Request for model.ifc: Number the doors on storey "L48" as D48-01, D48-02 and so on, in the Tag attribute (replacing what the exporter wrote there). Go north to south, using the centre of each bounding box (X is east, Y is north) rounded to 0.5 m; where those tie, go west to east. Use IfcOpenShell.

First a look at what the model holds.

```python
import ifcopenshell
import ifcopenshell.util.element
import ifcopenshell.util.placement

model = ifcopenshell.open("model.ifc")
print(model.schema)
storey = next(s for s in model.by_type("IfcBuildingStorey") if s.Name == "L48")
doors = [e for e in ifcopenshell.util.element.get_decomposition(storey) if e.is_a("IfcDoor")]
for e in sorted(doors, key=lambda e: e.id()):
    origin = ifcopenshell.util.placement.get_local_placement(e.ObjectPlacement)[:3, 3]
    print(e.id(), e.Tag, e.Name, origin.round(2) + 0.0, sep=" | ")
```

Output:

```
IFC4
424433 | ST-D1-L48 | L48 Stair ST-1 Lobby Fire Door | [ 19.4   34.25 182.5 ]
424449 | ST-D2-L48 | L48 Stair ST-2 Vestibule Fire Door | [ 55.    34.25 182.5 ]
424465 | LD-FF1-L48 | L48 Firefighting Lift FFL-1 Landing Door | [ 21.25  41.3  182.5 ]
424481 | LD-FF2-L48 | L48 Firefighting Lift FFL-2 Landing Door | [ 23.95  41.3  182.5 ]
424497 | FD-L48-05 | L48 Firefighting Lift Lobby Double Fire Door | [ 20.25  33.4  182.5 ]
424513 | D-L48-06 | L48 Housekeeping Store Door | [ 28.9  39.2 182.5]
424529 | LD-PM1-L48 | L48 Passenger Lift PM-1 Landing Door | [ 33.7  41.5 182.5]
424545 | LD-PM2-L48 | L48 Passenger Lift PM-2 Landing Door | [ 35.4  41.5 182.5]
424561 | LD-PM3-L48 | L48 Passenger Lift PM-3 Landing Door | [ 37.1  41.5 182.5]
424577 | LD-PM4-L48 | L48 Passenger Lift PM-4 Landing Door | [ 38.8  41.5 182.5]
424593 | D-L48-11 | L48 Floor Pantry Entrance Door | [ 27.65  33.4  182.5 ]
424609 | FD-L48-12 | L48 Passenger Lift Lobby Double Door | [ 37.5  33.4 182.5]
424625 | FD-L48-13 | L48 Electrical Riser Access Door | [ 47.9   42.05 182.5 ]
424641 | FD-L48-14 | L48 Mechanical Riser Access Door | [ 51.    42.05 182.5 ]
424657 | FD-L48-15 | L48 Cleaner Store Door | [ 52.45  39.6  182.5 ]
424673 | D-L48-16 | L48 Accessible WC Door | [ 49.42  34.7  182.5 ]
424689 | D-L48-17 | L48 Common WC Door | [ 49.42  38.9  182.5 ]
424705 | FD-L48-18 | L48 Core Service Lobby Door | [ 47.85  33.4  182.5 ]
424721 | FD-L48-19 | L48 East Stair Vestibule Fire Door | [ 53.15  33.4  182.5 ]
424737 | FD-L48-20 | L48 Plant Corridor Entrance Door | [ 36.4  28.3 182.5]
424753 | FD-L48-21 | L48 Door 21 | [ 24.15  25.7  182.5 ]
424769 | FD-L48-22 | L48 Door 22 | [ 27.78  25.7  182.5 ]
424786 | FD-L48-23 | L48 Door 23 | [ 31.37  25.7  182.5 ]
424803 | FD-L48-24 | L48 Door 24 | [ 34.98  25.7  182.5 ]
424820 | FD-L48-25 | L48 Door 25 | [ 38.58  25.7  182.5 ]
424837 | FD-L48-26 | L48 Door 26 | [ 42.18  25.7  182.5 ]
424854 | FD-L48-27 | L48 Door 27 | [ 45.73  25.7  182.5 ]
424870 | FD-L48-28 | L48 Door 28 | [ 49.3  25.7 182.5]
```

```python
import ifcopenshell
import ifcopenshell.geom
import ifcopenshell.util.element
import ifcopenshell.util.shape

model = ifcopenshell.open("model.ifc")
settings = ifcopenshell.geom.settings()
settings.set("use-world-coords", True)


def centre(element):
    shape = ifcopenshell.geom.create_shape(settings, element)
    return ifcopenshell.util.shape.get_bbox_centroid(shape.geometry)


storey = next(s for s in model.by_type("IfcBuildingStorey") if s.Name == "L48")
doors = [e for e in ifcopenshell.util.element.get_decomposition(storey) if e.is_a("IfcDoor")]

# Insertion points can sit at a corner or the storey origin, so sort by the geometry (in metres).
centres = {e: centre(e) for e in doors}
doors.sort(key=lambda e: (-round(centres[e][1] / 0.5), centres[e][0]))

for i, e in enumerate(doors, start=1):
    number = f"D48-{i:02d}"
    e.Tag = number
    print(e.id(), number)

model.write("model_updated.ifc")
```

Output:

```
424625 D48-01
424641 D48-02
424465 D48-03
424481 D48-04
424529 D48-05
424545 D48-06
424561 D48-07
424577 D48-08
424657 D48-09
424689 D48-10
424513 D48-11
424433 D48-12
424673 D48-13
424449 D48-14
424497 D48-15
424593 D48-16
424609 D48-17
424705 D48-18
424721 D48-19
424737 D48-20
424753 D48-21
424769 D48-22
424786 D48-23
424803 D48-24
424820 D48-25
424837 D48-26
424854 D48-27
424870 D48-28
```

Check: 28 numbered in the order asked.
